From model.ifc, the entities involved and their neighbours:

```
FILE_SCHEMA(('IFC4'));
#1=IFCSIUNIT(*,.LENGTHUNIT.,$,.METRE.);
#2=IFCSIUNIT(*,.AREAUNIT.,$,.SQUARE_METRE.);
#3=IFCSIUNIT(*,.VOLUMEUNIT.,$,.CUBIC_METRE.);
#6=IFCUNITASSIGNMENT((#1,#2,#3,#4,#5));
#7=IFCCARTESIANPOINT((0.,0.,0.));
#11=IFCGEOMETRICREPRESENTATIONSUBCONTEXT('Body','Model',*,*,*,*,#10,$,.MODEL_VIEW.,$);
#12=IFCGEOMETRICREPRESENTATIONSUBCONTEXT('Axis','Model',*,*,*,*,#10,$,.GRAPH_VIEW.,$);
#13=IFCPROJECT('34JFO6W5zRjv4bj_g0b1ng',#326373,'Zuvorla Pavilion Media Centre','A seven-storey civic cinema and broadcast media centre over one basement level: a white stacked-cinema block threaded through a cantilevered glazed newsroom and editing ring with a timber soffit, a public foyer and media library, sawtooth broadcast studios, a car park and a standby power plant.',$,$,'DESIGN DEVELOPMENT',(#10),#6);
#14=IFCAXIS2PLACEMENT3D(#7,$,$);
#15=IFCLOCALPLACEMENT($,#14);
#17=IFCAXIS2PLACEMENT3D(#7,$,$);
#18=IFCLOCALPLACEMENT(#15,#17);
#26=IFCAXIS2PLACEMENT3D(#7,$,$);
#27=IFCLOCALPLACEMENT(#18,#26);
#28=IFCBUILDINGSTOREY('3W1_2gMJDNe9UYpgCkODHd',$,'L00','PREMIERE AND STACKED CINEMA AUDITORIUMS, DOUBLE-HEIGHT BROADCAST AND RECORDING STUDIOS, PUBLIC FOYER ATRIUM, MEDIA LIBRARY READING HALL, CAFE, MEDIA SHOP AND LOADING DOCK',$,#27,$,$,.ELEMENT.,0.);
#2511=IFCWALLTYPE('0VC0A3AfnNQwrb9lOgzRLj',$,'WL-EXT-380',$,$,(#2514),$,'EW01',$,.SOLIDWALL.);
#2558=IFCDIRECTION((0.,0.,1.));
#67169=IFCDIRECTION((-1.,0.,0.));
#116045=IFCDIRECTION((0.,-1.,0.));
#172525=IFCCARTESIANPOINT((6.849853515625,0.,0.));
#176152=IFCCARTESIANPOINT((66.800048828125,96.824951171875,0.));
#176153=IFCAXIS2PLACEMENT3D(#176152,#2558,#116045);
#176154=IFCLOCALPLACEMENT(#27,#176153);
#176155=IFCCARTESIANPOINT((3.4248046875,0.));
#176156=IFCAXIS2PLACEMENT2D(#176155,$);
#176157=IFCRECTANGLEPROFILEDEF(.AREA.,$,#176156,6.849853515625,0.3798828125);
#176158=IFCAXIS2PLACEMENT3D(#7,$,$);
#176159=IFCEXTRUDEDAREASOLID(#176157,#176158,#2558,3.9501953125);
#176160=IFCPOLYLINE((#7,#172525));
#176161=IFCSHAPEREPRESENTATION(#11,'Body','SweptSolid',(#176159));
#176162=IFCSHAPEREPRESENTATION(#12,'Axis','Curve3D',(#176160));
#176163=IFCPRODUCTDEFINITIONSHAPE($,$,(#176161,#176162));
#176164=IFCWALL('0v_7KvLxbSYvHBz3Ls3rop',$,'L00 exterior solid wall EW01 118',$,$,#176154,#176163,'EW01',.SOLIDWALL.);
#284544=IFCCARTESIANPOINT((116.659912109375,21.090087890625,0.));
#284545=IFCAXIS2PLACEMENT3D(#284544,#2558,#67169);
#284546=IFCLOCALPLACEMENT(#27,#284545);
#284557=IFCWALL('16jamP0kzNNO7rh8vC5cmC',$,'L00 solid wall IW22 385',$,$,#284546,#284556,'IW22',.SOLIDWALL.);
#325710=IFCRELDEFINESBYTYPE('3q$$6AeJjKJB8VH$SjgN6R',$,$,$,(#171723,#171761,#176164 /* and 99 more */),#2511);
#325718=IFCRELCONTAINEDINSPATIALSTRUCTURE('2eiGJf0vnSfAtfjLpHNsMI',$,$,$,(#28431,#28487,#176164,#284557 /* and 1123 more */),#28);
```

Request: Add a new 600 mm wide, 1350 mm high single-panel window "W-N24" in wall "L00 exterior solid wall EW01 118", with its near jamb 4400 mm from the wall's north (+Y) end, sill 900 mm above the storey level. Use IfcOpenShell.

```python
import numpy as np
import ifcopenshell
import ifcopenshell.api.feature
import ifcopenshell.api.geometry
import ifcopenshell.api.root
import ifcopenshell.api.spatial
import ifcopenshell.geom
import ifcopenshell.util.element
import ifcopenshell.util.placement
import ifcopenshell.util.representation
import ifcopenshell.util.shape
import ifcopenshell.util.unit

model = ifcopenshell.open("model.ifc")
unit_scale = ifcopenshell.util.unit.calculate_unit_scale(model)
settings = ifcopenshell.geom.settings()


def volume(element):
    """Net volume in cubic metres, openings subtracted."""
    shape = ifcopenshell.geom.create_shape(settings, element)
    return ifcopenshell.util.shape.get_volume(shape.geometry)


wall = model.by_guid("0v_7KvLxbSYvHBz3Ls3rop")
storey = ifcopenshell.util.element.get_container(wall, ifc_class="IfcBuildingStorey")
context = ifcopenshell.util.representation.get_context(model, "Model", "Body", "MODEL_VIEW")
before = volume(wall)

width, height, from_end, sill = 0.6, 1.35, 4.4, 0.9  # metres

# The wall runs along its own X axis, and the end named is its -X end.
wall_shape = ifcopenshell.geom.create_shape(settings, wall)
x, y, z = ifcopenshell.util.shape.get_vertices(wall_shape.geometry).T
start = x.min() + from_end
face, thickness = float(y.min()), float(y.max() - y.min())
wall_matrix = ifcopenshell.util.placement.get_local_placement(wall.ObjectPlacement)
level = ifcopenshell.util.placement.get_local_placement(storey.ObjectPlacement)[2, 3]


def in_wall(x, y):
    """Placement at x, y metres in the wall's axes, at sill height."""
    matrix = wall_matrix.copy()
    matrix[:, 3] = wall_matrix @ np.array([x / unit_scale, y / unit_scale, 0.0, 1.0])
    matrix[2, 3] = level + sill / unit_scale
    return matrix


# Opening: a box that overshoots both wall faces by 50 mm.
opening = ifcopenshell.api.root.create_entity(model, ifc_class="IfcOpeningElement", predefined_type="OPENING")
box = ifcopenshell.api.geometry.add_wall_representation(
    model, context=context, length=width, height=height, thickness=thickness + 0.1
)
ifcopenshell.api.geometry.assign_representation(model, product=opening, representation=box)
ifcopenshell.api.geometry.edit_object_placement(model, product=opening, matrix=in_wall(start, face - 0.05), is_si=False)
ifcopenshell.api.feature.add_feature(model, feature=opening, element=wall)

window = ifcopenshell.api.root.create_entity(model, ifc_class="IfcWindow", name="W-N24", predefined_type="WINDOW")
window.OverallWidth, window.OverallHeight = width / unit_scale, height / unit_scale
window.PartitioningType = "SINGLE_PANEL"
body = ifcopenshell.api.geometry.add_window_representation(
    model,
    context=context,
    overall_width=window.OverallWidth,
    overall_height=window.OverallHeight,
    partition_type="SINGLE_PANEL",
)
ifcopenshell.api.geometry.assign_representation(model, product=window, representation=body)
ifcopenshell.api.spatial.assign_container(model, products=[window], relating_structure=storey)
ifcopenshell.api.feature.add_filling(model, opening=opening, element=window)

# Centre the window in the wall's thickness.
ifcopenshell.api.geometry.edit_object_placement(model, product=window, matrix=in_wall(start, face), is_si=False)
window_shape = ifcopenshell.geom.create_shape(settings, window)
depth = ifcopenshell.util.shape.get_vertices(window_shape.geometry)[:, 1]
offset = face + thickness / 2 - (depth.min() + depth.max()) / 2
ifcopenshell.api.geometry.edit_object_placement(model, product=window, matrix=in_wall(start, offset), is_si=False)

after = volume(wall)

print(f"wall volume {before:.3f} -> {after:.3f} m3")

model.write("model_updated.ifc")
```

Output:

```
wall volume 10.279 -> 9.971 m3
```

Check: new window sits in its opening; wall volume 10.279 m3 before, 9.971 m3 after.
